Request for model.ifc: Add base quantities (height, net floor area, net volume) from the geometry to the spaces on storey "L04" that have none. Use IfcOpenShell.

First a look at what the model holds.

```python
import ifcopenshell
import ifcopenshell.util.element
import ifcopenshell.util.unit

model = ifcopenshell.open("model.ifc")
print(model.schema)
for unit_type in ("LENGTHUNIT", "AREAUNIT", "VOLUMEUNIT"):
    print(unit_type, ifcopenshell.util.unit.calculate_unit_scale(model, unit_type))
storey = next(s for s in model.by_type("IfcBuildingStorey") if s.Name == "L04")
spaces = [e for e in ifcopenshell.util.element.get_decomposition(storey) if e.is_a("IfcSpace")]
for e in sorted(spaces, key=lambda e: e.id()):
    print(e.id(), e.is_a(), e.Name, list(ifcopenshell.util.element.get_psets(e, qtos_only=True)), sep=" | ")
```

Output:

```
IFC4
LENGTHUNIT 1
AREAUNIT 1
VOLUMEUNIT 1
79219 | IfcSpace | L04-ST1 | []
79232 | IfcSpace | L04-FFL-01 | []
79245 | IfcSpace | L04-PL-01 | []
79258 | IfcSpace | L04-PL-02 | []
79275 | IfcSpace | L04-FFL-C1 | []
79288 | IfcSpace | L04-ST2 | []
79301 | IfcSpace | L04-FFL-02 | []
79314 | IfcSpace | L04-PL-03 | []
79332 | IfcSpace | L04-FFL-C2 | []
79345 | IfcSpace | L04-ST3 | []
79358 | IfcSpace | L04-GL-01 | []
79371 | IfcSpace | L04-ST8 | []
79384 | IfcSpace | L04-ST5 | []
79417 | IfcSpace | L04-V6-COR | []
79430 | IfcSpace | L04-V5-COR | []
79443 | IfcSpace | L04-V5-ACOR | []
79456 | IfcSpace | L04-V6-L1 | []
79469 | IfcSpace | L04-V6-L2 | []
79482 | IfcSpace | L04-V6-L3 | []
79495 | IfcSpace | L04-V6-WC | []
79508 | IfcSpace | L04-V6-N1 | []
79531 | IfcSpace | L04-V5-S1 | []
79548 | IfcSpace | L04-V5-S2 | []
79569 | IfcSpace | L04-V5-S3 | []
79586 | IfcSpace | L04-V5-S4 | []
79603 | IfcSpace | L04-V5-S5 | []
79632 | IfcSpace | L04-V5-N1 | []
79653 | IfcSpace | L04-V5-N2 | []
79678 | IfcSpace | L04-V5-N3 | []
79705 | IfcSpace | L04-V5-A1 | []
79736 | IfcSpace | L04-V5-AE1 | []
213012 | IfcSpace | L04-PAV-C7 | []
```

```python
import ifcopenshell
import ifcopenshell.api.pset
import ifcopenshell.geom
import ifcopenshell.util.element
import ifcopenshell.util.shape
import ifcopenshell.util.unit

model = ifcopenshell.open("model.ifc")
unit_scale = ifcopenshell.util.unit.calculate_unit_scale(model)
area_scale = ifcopenshell.util.unit.calculate_unit_scale(model, "AREAUNIT")
volume_scale = ifcopenshell.util.unit.calculate_unit_scale(model, "VOLUMEUNIT")
settings = ifcopenshell.geom.settings()

storey = next(s for s in model.by_type("IfcBuildingStorey") if s.Name == "L04")
spaces = [e for e in ifcopenshell.util.element.get_decomposition(storey) if e.is_a("IfcSpace")]

for e in sorted(spaces, key=lambda e: e.id()):
    if ifcopenshell.util.element.get_psets(e, qtos_only=True, should_inherit=False):
        continue
    # Geometry comes back in metres, in the element's own axes.
    shape = ifcopenshell.geom.create_shape(settings, e)
    values = {
        "Height": ifcopenshell.util.shape.get_z(shape.geometry) / unit_scale,
        "NetFloorArea": ifcopenshell.util.shape.get_footprint_area(shape.geometry) / area_scale,
        "NetVolume": ifcopenshell.util.shape.get_volume(shape.geometry) / volume_scale,
    }
    qto = ifcopenshell.api.pset.add_qto(model, product=e, name="Qto_SpaceBaseQuantities")
    ifcopenshell.api.pset.edit_qto(model, qto=qto, properties=values)
    print(e.id(), {k: round(v, 3) for k, v in values.items()})

model.write("model_edited.ifc")
```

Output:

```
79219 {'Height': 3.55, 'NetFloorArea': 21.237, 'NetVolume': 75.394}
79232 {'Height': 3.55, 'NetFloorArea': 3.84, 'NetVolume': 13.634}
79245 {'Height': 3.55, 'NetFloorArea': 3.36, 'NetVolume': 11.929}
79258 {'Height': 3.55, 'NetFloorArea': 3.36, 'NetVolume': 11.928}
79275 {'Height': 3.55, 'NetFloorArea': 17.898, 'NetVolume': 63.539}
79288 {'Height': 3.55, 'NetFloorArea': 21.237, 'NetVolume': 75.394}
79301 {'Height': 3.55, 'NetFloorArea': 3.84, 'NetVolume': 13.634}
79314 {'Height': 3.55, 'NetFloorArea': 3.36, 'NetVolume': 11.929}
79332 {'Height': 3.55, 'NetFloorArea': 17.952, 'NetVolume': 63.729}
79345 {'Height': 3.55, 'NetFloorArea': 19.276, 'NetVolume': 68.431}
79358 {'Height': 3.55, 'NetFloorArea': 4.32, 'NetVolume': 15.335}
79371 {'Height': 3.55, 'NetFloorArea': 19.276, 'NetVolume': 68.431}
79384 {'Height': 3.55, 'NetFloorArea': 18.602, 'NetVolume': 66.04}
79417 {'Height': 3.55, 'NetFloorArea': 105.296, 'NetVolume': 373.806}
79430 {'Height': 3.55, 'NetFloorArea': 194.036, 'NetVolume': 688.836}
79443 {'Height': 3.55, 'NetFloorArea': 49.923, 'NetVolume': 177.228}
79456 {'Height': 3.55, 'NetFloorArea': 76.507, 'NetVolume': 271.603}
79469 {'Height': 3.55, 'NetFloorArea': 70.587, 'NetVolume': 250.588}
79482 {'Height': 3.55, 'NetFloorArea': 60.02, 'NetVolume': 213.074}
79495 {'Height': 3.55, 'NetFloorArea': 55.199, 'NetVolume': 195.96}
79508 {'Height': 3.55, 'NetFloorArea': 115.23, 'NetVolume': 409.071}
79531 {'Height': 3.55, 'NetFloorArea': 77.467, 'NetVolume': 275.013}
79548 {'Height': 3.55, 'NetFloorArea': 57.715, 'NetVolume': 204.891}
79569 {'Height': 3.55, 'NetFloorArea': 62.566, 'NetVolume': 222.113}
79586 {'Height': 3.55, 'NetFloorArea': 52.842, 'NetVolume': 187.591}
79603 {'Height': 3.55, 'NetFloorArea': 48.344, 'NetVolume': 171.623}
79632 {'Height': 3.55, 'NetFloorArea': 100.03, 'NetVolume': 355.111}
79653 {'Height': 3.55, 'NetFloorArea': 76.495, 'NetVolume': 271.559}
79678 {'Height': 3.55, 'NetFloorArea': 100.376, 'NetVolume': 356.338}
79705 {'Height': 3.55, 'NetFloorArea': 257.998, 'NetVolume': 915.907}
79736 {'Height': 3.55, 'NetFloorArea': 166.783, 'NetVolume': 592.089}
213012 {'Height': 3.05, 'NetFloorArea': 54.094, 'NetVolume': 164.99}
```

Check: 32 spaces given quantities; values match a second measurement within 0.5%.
